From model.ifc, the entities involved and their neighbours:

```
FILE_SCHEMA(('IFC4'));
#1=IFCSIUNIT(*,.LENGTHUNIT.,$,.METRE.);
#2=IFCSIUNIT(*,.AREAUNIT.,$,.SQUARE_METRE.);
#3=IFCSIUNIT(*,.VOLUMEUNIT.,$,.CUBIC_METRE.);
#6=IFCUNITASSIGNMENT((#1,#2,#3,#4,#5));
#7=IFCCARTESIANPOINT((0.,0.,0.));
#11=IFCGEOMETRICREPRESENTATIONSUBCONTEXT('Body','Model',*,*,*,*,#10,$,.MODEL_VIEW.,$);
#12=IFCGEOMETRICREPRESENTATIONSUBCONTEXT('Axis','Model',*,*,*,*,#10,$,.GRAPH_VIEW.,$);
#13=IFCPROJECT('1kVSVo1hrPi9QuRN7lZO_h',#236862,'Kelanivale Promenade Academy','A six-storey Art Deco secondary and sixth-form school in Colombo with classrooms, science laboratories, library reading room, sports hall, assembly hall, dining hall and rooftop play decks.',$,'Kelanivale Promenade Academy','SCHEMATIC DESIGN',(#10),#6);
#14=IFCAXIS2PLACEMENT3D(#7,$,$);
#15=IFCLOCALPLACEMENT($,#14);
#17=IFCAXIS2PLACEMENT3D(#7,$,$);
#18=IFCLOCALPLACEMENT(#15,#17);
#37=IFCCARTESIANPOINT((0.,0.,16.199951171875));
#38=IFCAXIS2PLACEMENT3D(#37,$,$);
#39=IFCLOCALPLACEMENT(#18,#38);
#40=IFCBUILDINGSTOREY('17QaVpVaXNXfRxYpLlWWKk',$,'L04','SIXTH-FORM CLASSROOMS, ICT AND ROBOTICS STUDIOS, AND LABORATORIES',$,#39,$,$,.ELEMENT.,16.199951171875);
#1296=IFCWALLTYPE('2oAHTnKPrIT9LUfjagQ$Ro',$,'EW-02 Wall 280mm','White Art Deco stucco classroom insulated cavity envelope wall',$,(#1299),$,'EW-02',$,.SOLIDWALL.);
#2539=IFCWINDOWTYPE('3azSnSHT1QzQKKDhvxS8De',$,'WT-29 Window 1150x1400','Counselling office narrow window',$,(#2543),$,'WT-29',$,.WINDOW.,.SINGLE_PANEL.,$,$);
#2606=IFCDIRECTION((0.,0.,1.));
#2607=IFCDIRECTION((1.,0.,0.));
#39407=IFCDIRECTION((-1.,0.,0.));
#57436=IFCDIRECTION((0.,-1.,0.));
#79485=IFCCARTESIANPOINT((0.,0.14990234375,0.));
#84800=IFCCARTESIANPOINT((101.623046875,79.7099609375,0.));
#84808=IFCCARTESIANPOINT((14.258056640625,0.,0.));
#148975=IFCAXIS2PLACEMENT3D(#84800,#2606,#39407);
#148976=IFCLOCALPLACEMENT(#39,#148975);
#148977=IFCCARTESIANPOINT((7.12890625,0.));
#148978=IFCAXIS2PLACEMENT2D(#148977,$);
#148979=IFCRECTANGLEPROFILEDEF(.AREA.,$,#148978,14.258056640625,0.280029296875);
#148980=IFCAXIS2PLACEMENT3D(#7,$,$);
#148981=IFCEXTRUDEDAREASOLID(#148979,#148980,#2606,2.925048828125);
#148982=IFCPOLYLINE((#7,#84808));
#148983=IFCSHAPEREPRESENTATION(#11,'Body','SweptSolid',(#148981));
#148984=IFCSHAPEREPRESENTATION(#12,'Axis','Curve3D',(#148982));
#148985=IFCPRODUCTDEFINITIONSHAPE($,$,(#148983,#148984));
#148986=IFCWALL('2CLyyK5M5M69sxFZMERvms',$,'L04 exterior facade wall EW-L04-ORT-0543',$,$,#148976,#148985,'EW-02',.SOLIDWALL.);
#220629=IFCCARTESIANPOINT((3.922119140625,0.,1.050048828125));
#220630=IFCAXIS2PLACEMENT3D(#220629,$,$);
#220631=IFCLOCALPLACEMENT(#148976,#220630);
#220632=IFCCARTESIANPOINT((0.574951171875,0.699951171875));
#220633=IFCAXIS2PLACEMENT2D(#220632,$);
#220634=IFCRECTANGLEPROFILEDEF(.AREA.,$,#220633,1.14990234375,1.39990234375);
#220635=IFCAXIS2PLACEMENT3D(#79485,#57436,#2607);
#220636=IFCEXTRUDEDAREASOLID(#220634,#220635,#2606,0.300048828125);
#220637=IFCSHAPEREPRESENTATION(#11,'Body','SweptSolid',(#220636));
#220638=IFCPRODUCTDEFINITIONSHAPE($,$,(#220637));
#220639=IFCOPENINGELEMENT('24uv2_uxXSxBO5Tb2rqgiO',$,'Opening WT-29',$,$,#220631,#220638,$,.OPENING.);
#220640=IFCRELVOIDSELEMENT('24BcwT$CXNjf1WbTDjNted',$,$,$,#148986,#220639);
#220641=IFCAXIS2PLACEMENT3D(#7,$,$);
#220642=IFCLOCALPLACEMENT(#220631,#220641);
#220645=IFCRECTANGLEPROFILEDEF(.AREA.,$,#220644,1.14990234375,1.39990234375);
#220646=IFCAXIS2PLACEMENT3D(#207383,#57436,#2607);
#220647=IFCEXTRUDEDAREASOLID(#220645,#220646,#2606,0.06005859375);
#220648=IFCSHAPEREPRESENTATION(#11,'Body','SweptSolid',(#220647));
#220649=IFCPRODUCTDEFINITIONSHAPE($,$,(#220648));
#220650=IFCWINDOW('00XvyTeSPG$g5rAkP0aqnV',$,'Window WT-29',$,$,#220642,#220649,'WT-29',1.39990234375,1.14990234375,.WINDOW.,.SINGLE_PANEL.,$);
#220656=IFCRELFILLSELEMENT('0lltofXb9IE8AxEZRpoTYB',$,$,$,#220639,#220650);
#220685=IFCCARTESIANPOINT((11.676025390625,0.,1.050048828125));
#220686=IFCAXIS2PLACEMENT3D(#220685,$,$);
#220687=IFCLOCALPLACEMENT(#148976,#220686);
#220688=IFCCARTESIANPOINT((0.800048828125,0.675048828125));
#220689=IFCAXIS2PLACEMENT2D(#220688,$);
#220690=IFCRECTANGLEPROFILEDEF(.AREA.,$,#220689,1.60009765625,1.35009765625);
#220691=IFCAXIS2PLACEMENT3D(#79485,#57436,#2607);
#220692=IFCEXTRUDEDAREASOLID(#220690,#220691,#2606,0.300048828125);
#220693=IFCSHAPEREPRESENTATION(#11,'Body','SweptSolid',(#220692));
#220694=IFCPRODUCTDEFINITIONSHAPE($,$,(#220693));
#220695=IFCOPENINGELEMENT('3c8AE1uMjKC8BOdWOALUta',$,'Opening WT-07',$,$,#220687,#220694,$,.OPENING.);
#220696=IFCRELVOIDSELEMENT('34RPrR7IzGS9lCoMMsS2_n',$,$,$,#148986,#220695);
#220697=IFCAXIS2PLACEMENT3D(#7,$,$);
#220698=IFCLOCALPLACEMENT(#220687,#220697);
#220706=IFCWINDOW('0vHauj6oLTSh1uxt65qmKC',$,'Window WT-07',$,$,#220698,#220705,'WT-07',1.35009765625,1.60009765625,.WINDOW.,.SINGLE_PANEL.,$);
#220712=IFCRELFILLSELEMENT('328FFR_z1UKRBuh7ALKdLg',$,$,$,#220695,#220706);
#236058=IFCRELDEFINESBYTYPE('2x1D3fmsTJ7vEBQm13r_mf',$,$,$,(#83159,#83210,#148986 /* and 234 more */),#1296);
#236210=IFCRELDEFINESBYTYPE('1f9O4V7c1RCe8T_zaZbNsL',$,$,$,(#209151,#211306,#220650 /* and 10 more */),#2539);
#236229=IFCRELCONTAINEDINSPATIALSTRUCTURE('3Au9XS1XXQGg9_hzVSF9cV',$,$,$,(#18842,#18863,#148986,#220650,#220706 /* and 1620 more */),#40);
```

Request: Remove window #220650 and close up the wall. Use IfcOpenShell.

```python
import ifcopenshell
import ifcopenshell.api.feature
import ifcopenshell.api.root
import ifcopenshell.geom
import ifcopenshell.util.shape

model = ifcopenshell.open("model.ifc")
settings = ifcopenshell.geom.settings()


def volume(element):
    """Net volume in cubic metres, openings subtracted."""
    shape = ifcopenshell.geom.create_shape(settings, element)
    return ifcopenshell.util.shape.get_volume(shape.geometry)


window = model.by_guid("00XvyTeSPG$g5rAkP0aqnV")
opening = window.FillsVoids[0].RelatingOpeningElement
wall = opening.VoidsElements[0].RelatingBuildingElement
before = volume(wall)

ifcopenshell.api.root.remove_product(model, product=window)
ifcopenshell.api.feature.remove_feature(model, feature=opening)

after = volume(wall)

print(f"wall volume {before:.3f} -> {after:.3f} m3")

model.write("model_rev.ifc")
```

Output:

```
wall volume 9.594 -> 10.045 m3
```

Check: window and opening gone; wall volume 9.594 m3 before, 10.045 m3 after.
